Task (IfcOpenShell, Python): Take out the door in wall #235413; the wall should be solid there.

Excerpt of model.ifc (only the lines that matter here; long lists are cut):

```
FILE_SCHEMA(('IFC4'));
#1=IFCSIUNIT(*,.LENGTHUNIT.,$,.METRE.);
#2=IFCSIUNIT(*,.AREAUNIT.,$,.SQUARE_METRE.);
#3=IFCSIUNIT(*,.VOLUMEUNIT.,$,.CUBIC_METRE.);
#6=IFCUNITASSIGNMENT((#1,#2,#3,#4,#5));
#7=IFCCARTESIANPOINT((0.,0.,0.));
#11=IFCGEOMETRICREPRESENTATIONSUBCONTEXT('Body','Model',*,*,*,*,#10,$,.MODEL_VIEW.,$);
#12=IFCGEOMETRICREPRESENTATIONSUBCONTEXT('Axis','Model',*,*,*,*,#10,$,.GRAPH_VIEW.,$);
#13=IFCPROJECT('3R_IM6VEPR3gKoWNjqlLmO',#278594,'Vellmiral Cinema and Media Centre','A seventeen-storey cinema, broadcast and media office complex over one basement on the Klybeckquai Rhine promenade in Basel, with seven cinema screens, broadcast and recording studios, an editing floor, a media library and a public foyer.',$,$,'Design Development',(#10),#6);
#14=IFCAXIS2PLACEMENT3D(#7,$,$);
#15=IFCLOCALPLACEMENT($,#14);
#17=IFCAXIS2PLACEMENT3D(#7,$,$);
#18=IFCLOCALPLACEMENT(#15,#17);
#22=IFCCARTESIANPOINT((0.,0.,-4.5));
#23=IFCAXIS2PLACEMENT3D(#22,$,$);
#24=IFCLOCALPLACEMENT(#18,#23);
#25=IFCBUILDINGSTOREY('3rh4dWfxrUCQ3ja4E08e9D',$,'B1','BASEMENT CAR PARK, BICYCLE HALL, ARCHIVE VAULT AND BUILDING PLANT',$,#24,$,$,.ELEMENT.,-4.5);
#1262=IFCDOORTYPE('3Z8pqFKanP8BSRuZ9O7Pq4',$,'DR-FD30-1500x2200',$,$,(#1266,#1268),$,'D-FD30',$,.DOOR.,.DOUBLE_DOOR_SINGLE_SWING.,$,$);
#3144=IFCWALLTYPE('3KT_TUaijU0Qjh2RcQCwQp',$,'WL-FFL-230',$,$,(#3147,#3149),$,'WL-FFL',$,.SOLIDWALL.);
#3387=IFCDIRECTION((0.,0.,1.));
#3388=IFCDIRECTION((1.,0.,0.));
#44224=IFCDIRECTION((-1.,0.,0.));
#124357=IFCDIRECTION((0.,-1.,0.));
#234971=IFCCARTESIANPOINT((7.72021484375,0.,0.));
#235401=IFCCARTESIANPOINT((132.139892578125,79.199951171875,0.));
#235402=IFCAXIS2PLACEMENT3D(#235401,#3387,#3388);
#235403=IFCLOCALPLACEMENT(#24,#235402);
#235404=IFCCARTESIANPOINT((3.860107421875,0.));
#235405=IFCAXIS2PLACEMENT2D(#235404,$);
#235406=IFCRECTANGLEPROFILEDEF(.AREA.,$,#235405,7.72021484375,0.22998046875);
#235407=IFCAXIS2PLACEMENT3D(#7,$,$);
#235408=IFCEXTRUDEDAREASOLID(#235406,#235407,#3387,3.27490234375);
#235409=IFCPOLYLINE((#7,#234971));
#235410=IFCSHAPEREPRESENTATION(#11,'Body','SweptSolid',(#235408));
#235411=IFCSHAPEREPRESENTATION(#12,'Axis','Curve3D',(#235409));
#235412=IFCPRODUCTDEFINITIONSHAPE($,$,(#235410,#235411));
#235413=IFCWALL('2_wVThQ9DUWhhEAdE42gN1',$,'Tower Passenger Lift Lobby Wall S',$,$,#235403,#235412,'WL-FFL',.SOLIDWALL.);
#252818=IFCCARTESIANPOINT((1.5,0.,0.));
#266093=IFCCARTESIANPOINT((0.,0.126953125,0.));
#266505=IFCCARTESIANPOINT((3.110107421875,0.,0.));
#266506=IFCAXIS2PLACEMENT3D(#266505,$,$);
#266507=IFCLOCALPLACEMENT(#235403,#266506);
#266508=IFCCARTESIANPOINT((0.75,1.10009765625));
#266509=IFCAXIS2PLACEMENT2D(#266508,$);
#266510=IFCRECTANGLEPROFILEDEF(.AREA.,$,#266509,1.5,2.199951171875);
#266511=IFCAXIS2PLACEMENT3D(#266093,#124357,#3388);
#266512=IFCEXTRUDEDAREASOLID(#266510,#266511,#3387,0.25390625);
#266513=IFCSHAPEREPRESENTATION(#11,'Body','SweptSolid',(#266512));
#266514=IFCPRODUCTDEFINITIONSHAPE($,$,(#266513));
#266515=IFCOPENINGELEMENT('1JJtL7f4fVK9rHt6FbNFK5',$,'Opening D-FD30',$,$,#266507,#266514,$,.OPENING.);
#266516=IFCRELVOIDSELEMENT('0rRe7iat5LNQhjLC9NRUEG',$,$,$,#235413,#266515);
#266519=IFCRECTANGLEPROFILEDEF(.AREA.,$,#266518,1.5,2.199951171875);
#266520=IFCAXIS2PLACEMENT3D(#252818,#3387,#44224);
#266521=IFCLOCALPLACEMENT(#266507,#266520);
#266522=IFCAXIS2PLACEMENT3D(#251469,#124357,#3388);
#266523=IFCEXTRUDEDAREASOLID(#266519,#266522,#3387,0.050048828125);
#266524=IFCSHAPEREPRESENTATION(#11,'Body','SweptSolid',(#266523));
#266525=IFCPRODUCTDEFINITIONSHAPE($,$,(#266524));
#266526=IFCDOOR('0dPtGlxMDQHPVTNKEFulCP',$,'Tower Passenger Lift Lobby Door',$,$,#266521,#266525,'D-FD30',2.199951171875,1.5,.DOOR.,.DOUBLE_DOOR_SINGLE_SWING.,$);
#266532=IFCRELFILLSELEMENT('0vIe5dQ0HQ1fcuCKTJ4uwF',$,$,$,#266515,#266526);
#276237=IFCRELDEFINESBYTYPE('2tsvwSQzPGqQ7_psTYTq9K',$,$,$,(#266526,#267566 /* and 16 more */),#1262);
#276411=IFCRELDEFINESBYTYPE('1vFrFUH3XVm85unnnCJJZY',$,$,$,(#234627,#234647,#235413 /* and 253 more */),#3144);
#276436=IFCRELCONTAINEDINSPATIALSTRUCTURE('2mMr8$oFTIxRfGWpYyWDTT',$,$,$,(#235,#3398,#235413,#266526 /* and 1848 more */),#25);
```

```python
import ifcopenshell
import ifcopenshell.api.feature
import ifcopenshell.api.root
import ifcopenshell.geom
import ifcopenshell.util.shape

model = ifcopenshell.open("model.ifc")
settings = ifcopenshell.geom.settings()


def volume(element):
    """Net volume in cubic metres, openings subtracted."""
    shape = ifcopenshell.geom.create_shape(settings, element)
    return ifcopenshell.util.shape.get_volume(shape.geometry)


door = model.by_guid("0dPtGlxMDQHPVTNKEFulCP")
opening = door.FillsVoids[0].RelatingOpeningElement
wall = opening.VoidsElements[0].RelatingBuildingElement
before = volume(wall)

ifcopenshell.api.root.remove_product(model, product=door)
ifcopenshell.api.feature.remove_feature(model, feature=opening)

after = volume(wall)

print(f"wall volume {before:.3f} -> {after:.3f} m3")

model.write("model_updated.ifc")
```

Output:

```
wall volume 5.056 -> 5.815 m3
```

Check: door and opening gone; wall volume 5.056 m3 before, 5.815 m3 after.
